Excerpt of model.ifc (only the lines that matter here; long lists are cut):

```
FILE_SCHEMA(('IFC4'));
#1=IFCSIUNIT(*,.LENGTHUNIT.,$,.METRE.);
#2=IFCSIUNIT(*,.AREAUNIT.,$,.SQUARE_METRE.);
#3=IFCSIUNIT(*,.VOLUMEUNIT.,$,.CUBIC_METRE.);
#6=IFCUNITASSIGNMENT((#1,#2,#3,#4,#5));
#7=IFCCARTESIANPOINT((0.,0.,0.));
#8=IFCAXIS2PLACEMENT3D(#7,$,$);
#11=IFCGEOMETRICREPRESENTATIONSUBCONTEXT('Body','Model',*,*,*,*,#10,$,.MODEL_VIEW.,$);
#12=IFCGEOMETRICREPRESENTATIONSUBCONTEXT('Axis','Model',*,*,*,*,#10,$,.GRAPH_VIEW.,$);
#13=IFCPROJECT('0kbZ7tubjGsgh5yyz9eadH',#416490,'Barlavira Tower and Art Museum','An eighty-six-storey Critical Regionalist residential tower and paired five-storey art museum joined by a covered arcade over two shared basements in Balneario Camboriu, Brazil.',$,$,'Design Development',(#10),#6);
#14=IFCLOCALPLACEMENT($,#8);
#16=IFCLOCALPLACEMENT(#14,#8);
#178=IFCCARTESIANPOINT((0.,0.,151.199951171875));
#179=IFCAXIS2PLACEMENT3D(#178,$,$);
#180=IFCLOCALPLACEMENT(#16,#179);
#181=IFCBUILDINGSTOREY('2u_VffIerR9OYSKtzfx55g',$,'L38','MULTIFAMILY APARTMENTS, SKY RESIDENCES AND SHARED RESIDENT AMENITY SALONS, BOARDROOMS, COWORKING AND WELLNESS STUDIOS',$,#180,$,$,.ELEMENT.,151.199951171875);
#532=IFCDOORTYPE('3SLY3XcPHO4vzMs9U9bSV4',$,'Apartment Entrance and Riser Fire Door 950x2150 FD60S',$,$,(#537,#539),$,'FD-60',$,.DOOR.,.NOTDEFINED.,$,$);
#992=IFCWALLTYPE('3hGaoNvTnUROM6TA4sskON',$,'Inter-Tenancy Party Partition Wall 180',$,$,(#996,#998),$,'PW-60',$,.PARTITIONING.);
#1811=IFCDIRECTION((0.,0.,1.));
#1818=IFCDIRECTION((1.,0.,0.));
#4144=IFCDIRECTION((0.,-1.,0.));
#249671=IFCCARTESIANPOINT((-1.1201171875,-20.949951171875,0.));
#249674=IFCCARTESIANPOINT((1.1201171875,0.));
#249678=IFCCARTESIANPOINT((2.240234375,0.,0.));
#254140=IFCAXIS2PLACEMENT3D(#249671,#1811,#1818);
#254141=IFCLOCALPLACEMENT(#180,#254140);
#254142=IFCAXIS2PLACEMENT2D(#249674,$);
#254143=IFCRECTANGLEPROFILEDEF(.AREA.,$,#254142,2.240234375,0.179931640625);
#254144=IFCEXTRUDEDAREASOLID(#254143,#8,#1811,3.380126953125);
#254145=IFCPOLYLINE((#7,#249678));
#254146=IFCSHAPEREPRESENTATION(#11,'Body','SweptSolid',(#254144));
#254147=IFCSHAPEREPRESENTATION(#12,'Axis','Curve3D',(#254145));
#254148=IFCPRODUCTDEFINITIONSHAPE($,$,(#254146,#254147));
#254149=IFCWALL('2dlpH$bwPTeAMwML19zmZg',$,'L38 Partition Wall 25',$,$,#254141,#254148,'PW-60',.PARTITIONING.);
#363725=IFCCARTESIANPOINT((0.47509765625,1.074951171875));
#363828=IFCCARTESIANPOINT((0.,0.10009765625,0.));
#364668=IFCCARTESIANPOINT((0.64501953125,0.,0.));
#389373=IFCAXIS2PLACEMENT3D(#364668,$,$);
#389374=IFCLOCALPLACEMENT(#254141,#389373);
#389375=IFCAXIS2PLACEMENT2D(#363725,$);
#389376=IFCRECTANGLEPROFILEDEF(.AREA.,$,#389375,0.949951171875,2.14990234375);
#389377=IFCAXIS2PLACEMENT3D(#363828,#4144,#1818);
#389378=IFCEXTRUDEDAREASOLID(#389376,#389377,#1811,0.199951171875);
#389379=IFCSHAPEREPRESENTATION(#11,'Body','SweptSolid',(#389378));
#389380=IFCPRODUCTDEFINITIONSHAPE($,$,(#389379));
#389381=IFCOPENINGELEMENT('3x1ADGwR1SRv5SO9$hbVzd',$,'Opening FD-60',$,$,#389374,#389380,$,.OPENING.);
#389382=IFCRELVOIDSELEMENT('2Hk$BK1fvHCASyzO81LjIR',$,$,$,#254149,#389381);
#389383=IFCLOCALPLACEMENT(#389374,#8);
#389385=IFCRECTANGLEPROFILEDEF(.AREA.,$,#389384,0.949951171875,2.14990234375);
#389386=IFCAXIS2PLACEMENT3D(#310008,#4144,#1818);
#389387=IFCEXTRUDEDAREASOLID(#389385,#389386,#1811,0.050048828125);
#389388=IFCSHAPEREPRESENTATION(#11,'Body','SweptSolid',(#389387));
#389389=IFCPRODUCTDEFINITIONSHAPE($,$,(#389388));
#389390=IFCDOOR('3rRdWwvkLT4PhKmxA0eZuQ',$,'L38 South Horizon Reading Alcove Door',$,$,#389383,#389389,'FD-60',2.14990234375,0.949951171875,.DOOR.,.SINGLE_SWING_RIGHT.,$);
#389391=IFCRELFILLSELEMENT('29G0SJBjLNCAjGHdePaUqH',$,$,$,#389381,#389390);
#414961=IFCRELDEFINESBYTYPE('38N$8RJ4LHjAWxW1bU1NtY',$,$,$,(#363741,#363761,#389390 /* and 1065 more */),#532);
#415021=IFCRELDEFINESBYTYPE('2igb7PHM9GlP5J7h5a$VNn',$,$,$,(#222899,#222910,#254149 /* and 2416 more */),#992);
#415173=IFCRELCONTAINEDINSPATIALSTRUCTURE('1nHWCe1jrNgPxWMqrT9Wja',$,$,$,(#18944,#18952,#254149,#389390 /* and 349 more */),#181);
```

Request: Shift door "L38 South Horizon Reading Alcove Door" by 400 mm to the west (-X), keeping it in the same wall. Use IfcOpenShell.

```python
import ifcopenshell
import ifcopenshell.api.geometry
import ifcopenshell.util.placement
import ifcopenshell.util.unit

model = ifcopenshell.open("model.ifc")
unit_scale = ifcopenshell.util.unit.calculate_unit_scale(model)

door = model.by_guid("3rRdWwvkLT4PhKmxA0eZuQ")
opening = door.FillsVoids[0].RelatingOpeningElement
wall = opening.VoidsElements[0].RelatingBuildingElement

wall_matrix = ifcopenshell.util.placement.get_local_placement(wall.ObjectPlacement)
shift = wall_matrix[:3, 0] * -0.4 / unit_scale
before = ifcopenshell.util.placement.get_local_placement(door.ObjectPlacement)[:3, 3].copy()

# The door is placed relative to its opening, so it follows when the opening moves.
matrix = ifcopenshell.util.placement.get_local_placement(opening.ObjectPlacement)
matrix[:3, 3] += shift
ifcopenshell.api.geometry.edit_object_placement(
    model, product=opening, matrix=matrix, is_si=False, should_transform_children=True
)

after = ifcopenshell.util.placement.get_local_placement(door.ObjectPlacement)[:3, 3]
print("door moved by", (after - before).round(3) + 0.0)

model.write("model-out.ifc")
```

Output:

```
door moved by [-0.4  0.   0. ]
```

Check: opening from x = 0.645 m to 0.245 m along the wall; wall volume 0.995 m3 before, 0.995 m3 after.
